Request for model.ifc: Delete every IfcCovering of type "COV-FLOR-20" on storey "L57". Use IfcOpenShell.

First a look at what the model holds.

```python
import ifcopenshell
import ifcopenshell.util.element

model = ifcopenshell.open("model.ifc")
print(model.schema)
storey = next(s for s in model.by_type("IfcBuildingStorey") if s.Name == "L57")
coverings = [e for e in ifcopenshell.util.element.get_decomposition(storey) if e.is_a("IfcCovering")]
seen = {}
for e in coverings:
    element_type = ifcopenshell.util.element.get_type(e)
    name = element_type.Name if element_type not in (None, e) else None
    seen[name] = seen.get(name, 0) + 1
for name, count in sorted(seen.items(), key=str):
    print(count, "x", name)
```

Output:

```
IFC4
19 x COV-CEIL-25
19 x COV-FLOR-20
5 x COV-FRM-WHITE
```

```python
import ifcopenshell
import ifcopenshell.api.root
import ifcopenshell.util.element

model = ifcopenshell.open("model.ifc")

storey = next(s for s in model.by_type("IfcBuildingStorey") if s.Name == "L57")
coverings = [e for e in ifcopenshell.util.element.get_decomposition(storey) if e.is_a("IfcCovering")]
targets = [e for e in coverings if (t := ifcopenshell.util.element.get_type(e)) not in (None, e) and t.Name == "COV-FLOR-20"]

for e in targets:
    ifcopenshell.api.root.remove_product(model, product=e)
print(len(targets), "removed")

model.write("model_updated.ifc")
```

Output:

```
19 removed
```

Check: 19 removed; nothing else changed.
